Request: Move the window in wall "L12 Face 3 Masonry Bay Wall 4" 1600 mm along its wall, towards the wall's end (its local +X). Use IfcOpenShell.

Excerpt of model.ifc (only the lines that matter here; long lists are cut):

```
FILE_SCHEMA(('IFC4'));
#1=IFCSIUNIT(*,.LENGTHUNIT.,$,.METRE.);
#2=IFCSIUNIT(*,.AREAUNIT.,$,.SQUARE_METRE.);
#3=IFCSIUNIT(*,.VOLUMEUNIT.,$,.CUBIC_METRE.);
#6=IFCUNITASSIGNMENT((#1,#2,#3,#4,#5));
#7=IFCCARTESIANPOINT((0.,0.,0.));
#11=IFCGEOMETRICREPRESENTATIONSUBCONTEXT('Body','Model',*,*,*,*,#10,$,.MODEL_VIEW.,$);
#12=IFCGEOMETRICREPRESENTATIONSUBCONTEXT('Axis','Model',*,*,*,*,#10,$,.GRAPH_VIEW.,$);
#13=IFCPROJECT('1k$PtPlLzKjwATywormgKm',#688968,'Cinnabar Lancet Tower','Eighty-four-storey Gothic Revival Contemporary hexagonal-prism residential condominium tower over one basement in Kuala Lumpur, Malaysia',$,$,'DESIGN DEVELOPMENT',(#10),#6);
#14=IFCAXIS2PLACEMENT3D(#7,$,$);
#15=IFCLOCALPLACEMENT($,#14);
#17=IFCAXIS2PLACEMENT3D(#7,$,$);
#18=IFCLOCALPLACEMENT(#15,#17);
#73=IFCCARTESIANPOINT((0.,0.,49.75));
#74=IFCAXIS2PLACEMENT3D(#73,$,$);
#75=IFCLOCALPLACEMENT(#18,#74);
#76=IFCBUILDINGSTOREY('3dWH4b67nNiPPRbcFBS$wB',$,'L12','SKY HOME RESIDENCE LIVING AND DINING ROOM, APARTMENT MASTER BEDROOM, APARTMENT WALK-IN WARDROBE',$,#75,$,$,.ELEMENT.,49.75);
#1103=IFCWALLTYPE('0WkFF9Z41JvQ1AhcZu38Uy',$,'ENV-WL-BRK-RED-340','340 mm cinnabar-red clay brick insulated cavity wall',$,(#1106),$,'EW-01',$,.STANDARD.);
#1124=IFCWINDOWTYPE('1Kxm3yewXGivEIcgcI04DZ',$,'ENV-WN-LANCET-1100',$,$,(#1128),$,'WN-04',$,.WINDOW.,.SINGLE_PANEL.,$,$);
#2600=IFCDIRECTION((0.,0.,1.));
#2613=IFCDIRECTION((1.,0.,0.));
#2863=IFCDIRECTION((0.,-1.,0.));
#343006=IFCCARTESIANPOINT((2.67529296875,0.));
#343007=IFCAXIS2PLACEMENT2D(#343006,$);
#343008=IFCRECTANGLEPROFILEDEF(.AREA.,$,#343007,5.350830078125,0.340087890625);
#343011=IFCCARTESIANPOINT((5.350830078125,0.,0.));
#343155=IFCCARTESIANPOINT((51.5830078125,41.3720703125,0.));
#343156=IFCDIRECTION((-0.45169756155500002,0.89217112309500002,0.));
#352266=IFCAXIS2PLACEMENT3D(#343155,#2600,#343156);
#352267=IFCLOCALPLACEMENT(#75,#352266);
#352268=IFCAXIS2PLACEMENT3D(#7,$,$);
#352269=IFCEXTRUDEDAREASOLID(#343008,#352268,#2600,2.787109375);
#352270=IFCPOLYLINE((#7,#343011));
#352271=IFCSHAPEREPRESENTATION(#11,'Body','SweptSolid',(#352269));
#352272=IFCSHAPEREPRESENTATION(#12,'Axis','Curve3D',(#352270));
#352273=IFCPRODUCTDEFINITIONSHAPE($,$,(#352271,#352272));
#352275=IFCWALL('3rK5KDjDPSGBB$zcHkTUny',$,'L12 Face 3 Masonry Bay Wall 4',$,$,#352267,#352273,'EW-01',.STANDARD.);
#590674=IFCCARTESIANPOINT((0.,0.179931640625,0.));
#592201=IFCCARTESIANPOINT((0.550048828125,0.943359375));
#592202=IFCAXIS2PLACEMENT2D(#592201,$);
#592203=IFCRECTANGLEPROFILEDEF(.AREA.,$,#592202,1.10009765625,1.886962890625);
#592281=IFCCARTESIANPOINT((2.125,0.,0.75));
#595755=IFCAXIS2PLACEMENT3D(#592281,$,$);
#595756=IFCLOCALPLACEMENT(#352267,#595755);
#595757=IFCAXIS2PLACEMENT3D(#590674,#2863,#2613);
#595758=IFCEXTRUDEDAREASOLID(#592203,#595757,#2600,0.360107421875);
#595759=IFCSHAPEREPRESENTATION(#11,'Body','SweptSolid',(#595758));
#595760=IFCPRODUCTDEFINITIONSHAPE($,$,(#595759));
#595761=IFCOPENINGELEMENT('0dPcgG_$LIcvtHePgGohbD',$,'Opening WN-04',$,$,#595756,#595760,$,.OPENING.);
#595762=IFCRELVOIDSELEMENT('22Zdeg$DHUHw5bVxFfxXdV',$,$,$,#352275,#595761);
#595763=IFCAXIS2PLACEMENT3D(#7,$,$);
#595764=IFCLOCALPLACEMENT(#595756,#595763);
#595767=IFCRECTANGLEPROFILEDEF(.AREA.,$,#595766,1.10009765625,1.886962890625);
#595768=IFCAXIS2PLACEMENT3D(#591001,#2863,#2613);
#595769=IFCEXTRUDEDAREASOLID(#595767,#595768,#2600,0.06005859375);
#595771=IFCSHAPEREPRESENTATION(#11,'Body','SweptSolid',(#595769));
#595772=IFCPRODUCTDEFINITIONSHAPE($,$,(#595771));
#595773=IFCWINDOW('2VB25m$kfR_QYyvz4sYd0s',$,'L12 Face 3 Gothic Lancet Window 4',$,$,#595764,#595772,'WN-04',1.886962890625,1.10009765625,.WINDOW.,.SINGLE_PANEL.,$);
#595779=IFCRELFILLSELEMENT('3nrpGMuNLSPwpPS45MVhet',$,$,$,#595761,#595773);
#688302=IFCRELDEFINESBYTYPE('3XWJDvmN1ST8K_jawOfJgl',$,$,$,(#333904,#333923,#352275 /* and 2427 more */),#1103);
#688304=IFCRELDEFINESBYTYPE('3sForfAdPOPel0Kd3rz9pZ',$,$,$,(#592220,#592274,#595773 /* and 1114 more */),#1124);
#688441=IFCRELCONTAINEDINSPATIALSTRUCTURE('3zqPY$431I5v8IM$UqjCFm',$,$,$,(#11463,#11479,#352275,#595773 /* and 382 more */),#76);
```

```python
import ifcopenshell
import ifcopenshell.api.geometry
import ifcopenshell.util.placement

model = ifcopenshell.open("model.ifc")

window = model.by_id(595773)
opening = window.FillsVoids[0].RelatingOpeningElement
wall = opening.VoidsElements[0].RelatingBuildingElement

wall_matrix = ifcopenshell.util.placement.get_local_placement(wall.ObjectPlacement)
shift = wall_matrix[:3, 0] * 1.6
before = ifcopenshell.util.placement.get_local_placement(window.ObjectPlacement)[:3, 3].copy()

# The window is placed relative to its opening, so it follows when the opening moves.
matrix = ifcopenshell.util.placement.get_local_placement(opening.ObjectPlacement)
matrix[:3, 3] += shift
ifcopenshell.api.geometry.edit_object_placement(
    model, product=opening, matrix=matrix, is_si=False, should_transform_children=True
)

after = ifcopenshell.util.placement.get_local_placement(window.ObjectPlacement)[:3, 3]
print("window moved by", (after - before).round(3) + 0.0)

model.write("model_v2.ifc")
```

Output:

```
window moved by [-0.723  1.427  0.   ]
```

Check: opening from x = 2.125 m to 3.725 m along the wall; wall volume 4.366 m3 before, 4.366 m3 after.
